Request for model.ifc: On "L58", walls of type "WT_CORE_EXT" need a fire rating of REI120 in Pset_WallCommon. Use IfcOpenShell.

First a look at what the model holds.

```python
import ifcopenshell
import ifcopenshell.util.element

model = ifcopenshell.open("model.ifc")
print(model.schema)
storey = next(s for s in model.by_type("IfcBuildingStorey") if s.Name == "L58")
walls = [e for e in ifcopenshell.util.element.get_decomposition(storey) if e.is_a("IfcWall")]
seen = {}
for e in walls:
    element_type = ifcopenshell.util.element.get_type(e)
    key = (element_type.Name if element_type != e and element_type else None, ifcopenshell.util.element.get_pset(e, "Pset_WallCommon", "FireRating"))
    seen[key] = seen.get(key, 0) + 1
for (name, value), count in sorted(seen.items(), key=str):
    print(count, "x", name, "|", value)
```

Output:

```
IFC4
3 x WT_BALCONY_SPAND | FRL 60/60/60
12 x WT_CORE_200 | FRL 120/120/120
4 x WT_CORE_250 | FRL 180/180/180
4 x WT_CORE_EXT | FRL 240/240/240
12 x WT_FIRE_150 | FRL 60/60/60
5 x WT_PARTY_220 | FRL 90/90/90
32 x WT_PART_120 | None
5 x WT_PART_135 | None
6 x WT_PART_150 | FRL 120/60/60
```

```python
import ifcopenshell
import ifcopenshell.api.pset
import ifcopenshell.util.element

model = ifcopenshell.open("model.ifc")

storey = next(s for s in model.by_type("IfcBuildingStorey") if s.Name == "L58")
walls = [e for e in ifcopenshell.util.element.get_decomposition(storey) if e.is_a("IfcWall")]

count = 0
for e in walls:
    element_type = ifcopenshell.util.element.get_type(e)
    if element_type in (None, e) or element_type.Name != "WT_CORE_EXT":
        continue
    found = ifcopenshell.util.element.get_pset(e, "Pset_WallCommon", should_inherit=False)
    if found:
        pset = model.by_id(found["id"])
        if len(ifcopenshell.util.element.get_elements_by_pset(pset)) > 1:
            pset = ifcopenshell.api.pset.unshare_pset(model, products=[e], pset=pset)[0]
    else:
        pset = ifcopenshell.api.pset.add_pset(model, product=e, name="Pset_WallCommon")
    ifcopenshell.api.pset.edit_pset(model, pset=pset, properties={"FireRating": "REI120"})
    count += 1

print(count, "walls updated")

model.write("model_updated.ifc")
```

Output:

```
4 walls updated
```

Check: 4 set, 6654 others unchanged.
